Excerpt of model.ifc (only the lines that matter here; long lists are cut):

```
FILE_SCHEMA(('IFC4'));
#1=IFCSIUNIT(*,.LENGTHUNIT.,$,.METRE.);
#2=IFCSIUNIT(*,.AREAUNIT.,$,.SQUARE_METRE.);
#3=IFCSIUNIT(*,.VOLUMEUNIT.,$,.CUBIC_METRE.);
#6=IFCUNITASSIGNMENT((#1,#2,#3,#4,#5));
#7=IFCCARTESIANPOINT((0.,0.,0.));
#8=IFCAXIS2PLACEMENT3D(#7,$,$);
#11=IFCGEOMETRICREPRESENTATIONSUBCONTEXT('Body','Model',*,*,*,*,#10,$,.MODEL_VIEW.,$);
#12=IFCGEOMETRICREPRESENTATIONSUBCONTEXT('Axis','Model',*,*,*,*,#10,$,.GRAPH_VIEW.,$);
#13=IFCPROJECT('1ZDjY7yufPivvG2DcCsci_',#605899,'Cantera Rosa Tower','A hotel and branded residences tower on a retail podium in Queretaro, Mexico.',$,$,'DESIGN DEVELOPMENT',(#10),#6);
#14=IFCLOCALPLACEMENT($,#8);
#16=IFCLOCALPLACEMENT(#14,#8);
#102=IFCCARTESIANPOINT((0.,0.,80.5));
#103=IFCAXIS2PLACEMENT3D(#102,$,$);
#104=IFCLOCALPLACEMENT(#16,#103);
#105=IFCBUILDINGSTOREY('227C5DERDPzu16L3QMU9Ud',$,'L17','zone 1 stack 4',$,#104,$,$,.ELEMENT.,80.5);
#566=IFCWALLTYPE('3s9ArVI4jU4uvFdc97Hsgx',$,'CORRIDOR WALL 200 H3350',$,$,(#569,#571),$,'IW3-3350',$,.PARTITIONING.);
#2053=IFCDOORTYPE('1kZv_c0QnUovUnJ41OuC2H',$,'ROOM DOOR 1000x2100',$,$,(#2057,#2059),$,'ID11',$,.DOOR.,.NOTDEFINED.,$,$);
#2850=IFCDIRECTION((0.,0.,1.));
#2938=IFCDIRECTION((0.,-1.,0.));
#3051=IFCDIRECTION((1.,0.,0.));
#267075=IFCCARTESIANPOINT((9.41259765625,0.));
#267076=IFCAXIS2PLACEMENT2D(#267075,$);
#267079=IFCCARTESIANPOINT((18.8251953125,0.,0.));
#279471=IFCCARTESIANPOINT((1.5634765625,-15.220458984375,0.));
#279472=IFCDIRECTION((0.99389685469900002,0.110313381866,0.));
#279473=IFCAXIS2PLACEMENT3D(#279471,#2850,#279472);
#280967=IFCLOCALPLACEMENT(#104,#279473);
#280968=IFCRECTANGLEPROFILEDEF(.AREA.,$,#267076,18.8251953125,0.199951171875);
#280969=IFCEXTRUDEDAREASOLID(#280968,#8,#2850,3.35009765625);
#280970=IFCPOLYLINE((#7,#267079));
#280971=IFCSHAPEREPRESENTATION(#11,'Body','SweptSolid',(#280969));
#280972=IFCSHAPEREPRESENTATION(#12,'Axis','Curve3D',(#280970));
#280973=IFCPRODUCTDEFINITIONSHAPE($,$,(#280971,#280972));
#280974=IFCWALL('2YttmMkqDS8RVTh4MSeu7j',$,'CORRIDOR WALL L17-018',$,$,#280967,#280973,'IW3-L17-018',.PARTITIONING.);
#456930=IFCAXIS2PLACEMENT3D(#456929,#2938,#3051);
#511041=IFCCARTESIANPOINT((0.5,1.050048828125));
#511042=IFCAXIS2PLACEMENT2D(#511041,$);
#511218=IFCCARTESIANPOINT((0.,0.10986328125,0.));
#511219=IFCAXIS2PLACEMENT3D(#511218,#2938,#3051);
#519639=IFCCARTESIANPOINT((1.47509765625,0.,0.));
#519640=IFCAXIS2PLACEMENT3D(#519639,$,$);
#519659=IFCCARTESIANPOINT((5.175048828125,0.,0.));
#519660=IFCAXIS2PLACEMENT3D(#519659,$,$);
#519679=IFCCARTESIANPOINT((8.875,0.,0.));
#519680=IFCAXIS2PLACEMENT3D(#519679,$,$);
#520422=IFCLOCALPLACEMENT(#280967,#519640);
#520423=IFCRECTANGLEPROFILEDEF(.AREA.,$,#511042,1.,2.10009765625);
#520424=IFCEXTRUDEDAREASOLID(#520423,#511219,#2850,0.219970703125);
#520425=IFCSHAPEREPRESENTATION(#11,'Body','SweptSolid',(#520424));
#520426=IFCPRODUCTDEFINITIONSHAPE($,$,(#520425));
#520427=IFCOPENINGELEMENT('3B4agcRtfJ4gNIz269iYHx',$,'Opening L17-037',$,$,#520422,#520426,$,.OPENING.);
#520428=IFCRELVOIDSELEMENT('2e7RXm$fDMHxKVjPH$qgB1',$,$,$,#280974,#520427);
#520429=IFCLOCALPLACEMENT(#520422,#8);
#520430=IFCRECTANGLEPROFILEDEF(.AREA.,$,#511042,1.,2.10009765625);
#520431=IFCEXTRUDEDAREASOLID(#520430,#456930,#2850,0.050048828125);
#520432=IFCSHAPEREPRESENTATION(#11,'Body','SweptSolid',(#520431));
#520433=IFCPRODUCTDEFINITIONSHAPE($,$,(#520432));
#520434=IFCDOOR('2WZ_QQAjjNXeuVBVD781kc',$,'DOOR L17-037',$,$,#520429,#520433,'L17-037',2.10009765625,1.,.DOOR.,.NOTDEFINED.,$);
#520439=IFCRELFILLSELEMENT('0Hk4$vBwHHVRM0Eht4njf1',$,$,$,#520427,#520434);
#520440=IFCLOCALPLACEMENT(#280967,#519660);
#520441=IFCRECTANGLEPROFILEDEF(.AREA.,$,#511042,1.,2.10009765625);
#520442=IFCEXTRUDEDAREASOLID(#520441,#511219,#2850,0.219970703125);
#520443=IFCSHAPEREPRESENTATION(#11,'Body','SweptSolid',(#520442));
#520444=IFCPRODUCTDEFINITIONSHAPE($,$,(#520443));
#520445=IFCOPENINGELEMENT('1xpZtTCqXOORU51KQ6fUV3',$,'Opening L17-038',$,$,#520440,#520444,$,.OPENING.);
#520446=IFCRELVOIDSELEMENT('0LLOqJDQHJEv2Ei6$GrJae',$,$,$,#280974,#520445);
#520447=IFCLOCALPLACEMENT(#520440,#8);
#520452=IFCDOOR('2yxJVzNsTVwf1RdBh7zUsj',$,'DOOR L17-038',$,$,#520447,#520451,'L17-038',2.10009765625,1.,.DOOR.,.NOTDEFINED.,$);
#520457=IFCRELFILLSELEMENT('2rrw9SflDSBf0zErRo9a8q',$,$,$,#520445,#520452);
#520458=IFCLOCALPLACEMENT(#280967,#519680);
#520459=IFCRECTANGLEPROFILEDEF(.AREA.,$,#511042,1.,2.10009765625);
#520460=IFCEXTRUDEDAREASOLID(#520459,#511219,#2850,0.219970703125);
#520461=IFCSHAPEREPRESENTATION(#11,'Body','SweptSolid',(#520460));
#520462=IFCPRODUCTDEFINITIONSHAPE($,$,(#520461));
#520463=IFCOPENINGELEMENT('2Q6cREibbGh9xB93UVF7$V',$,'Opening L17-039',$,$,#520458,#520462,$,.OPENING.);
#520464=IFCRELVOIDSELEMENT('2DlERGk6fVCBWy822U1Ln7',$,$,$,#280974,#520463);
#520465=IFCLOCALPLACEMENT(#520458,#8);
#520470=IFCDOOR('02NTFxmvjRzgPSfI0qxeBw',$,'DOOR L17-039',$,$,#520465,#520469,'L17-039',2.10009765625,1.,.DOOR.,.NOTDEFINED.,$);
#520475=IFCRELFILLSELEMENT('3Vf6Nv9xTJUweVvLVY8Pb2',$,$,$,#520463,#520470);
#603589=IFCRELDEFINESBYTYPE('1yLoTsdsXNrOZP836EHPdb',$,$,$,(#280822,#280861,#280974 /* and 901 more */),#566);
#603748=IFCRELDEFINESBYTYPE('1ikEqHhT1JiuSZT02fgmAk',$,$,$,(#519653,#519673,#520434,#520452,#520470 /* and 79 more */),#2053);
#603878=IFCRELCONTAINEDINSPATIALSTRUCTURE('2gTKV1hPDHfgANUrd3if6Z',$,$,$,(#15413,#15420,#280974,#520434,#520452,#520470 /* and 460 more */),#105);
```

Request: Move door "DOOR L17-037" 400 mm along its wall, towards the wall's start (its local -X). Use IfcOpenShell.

```python
import ifcopenshell
import ifcopenshell.api.geometry
import ifcopenshell.util.placement
import ifcopenshell.util.unit

model = ifcopenshell.open("model.ifc")
unit_scale = ifcopenshell.util.unit.calculate_unit_scale(model)

door = model.by_guid("2WZ_QQAjjNXeuVBVD781kc")
opening = door.FillsVoids[0].RelatingOpeningElement
wall = opening.VoidsElements[0].RelatingBuildingElement

wall_matrix = ifcopenshell.util.placement.get_local_placement(wall.ObjectPlacement)
shift = wall_matrix[:3, 0] * -0.4 / unit_scale
before = ifcopenshell.util.placement.get_local_placement(door.ObjectPlacement)[:3, 3].copy()

# The door is placed relative to its opening, so it follows when the opening moves.
matrix = ifcopenshell.util.placement.get_local_placement(opening.ObjectPlacement)
matrix[:3, 3] += shift
ifcopenshell.api.geometry.edit_object_placement(
    model, product=opening, matrix=matrix, is_si=False, should_transform_children=True
)

after = ifcopenshell.util.placement.get_local_placement(door.ObjectPlacement)[:3, 3]
print("door moved by", (after - before).round(3) + 0.0)

model.write("model_rev.ifc")
```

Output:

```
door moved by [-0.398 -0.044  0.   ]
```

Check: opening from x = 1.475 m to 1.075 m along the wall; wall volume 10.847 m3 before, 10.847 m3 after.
